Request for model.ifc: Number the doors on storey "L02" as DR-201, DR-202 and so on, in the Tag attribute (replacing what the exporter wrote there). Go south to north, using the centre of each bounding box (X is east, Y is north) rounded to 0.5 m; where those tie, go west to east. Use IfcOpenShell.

First a look at what the model holds.

```python
import ifcopenshell
import ifcopenshell.util.element
import ifcopenshell.util.placement

model = ifcopenshell.open("model.ifc")
print(model.schema)
storey = next(s for s in model.by_type("IfcBuildingStorey") if s.Name == "L02")
doors = [e for e in ifcopenshell.util.element.get_decomposition(storey) if e.is_a("IfcDoor")]
for e in sorted(doors, key=lambda e: e.id()):
    origin = ifcopenshell.util.placement.get_local_placement(e.ObjectPlacement)[:3, 3]
    print(e.id(), e.Tag, e.Name, origin.round(2) + 0.0, sep=" | ")
```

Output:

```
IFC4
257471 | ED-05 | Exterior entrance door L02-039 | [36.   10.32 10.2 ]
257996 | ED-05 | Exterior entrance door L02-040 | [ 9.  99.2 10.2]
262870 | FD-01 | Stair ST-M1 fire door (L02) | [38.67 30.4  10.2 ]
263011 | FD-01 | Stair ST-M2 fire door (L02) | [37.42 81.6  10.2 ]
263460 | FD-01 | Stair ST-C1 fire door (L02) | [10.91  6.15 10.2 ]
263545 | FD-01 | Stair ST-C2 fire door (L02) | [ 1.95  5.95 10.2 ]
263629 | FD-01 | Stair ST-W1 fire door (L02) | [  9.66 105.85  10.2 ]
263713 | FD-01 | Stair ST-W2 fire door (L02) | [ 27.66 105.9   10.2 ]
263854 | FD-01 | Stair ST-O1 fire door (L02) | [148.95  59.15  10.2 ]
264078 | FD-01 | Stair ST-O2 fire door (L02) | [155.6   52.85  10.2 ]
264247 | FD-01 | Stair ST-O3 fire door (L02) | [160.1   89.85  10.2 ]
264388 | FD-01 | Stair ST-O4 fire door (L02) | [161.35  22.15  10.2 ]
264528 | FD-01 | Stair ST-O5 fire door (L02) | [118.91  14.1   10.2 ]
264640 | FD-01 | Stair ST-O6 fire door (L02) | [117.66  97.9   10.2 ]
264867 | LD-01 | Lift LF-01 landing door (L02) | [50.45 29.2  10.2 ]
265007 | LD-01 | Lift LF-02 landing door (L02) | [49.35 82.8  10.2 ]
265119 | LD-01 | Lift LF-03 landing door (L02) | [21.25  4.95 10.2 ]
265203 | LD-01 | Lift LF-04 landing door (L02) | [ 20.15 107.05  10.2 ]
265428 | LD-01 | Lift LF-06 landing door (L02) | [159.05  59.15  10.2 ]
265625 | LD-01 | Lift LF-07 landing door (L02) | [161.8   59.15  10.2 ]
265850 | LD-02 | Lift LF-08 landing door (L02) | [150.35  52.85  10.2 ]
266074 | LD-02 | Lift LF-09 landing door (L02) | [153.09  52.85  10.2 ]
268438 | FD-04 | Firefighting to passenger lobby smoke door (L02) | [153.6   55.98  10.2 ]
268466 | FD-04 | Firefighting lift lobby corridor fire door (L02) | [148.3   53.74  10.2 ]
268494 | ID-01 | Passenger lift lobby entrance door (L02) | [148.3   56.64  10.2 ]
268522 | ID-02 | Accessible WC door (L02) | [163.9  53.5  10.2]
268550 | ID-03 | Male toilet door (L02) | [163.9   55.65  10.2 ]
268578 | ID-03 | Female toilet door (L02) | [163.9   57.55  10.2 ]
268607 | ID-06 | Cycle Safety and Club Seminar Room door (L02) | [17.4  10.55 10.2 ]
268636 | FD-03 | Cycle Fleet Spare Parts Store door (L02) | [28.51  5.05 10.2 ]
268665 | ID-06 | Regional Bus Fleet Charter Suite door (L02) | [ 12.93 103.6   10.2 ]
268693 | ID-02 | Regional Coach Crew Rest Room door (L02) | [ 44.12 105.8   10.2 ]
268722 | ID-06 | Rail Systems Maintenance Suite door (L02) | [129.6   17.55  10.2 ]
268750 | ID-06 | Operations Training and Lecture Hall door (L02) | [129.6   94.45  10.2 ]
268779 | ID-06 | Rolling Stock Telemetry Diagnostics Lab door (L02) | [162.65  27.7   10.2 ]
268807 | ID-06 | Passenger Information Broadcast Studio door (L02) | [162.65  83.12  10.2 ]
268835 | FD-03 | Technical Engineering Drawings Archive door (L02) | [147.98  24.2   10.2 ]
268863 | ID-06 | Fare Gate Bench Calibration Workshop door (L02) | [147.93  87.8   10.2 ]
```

```python
import ifcopenshell
import ifcopenshell.geom
import ifcopenshell.util.element
import ifcopenshell.util.shape

model = ifcopenshell.open("model.ifc")
settings = ifcopenshell.geom.settings()
settings.set("use-world-coords", True)


def centre(element):
    shape = ifcopenshell.geom.create_shape(settings, element)
    return ifcopenshell.util.shape.get_bbox_centroid(shape.geometry)


storey = next(s for s in model.by_type("IfcBuildingStorey") if s.Name == "L02")
doors = [e for e in ifcopenshell.util.element.get_decomposition(storey) if e.is_a("IfcDoor")]

# Insertion points can sit at a corner or the storey origin, so sort by the geometry (in metres).
centres = {e: centre(e) for e in doors}
doors.sort(key=lambda e: (round(centres[e][1] / 0.5), centres[e][0]))

for i, e in enumerate(doors, start=1):
    number = f"DR-2{i:02d}"
    e.Tag = number
    print(e.id(), number)

model.write("model-out.ifc")
```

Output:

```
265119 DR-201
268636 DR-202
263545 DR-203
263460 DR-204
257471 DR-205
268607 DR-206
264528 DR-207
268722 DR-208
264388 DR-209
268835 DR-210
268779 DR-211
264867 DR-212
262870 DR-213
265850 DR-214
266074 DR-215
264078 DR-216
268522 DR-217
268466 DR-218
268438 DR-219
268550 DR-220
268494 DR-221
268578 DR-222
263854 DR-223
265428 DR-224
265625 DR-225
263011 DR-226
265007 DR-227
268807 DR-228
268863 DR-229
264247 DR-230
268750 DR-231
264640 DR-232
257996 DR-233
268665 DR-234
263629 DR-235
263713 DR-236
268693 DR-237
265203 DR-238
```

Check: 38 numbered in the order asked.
